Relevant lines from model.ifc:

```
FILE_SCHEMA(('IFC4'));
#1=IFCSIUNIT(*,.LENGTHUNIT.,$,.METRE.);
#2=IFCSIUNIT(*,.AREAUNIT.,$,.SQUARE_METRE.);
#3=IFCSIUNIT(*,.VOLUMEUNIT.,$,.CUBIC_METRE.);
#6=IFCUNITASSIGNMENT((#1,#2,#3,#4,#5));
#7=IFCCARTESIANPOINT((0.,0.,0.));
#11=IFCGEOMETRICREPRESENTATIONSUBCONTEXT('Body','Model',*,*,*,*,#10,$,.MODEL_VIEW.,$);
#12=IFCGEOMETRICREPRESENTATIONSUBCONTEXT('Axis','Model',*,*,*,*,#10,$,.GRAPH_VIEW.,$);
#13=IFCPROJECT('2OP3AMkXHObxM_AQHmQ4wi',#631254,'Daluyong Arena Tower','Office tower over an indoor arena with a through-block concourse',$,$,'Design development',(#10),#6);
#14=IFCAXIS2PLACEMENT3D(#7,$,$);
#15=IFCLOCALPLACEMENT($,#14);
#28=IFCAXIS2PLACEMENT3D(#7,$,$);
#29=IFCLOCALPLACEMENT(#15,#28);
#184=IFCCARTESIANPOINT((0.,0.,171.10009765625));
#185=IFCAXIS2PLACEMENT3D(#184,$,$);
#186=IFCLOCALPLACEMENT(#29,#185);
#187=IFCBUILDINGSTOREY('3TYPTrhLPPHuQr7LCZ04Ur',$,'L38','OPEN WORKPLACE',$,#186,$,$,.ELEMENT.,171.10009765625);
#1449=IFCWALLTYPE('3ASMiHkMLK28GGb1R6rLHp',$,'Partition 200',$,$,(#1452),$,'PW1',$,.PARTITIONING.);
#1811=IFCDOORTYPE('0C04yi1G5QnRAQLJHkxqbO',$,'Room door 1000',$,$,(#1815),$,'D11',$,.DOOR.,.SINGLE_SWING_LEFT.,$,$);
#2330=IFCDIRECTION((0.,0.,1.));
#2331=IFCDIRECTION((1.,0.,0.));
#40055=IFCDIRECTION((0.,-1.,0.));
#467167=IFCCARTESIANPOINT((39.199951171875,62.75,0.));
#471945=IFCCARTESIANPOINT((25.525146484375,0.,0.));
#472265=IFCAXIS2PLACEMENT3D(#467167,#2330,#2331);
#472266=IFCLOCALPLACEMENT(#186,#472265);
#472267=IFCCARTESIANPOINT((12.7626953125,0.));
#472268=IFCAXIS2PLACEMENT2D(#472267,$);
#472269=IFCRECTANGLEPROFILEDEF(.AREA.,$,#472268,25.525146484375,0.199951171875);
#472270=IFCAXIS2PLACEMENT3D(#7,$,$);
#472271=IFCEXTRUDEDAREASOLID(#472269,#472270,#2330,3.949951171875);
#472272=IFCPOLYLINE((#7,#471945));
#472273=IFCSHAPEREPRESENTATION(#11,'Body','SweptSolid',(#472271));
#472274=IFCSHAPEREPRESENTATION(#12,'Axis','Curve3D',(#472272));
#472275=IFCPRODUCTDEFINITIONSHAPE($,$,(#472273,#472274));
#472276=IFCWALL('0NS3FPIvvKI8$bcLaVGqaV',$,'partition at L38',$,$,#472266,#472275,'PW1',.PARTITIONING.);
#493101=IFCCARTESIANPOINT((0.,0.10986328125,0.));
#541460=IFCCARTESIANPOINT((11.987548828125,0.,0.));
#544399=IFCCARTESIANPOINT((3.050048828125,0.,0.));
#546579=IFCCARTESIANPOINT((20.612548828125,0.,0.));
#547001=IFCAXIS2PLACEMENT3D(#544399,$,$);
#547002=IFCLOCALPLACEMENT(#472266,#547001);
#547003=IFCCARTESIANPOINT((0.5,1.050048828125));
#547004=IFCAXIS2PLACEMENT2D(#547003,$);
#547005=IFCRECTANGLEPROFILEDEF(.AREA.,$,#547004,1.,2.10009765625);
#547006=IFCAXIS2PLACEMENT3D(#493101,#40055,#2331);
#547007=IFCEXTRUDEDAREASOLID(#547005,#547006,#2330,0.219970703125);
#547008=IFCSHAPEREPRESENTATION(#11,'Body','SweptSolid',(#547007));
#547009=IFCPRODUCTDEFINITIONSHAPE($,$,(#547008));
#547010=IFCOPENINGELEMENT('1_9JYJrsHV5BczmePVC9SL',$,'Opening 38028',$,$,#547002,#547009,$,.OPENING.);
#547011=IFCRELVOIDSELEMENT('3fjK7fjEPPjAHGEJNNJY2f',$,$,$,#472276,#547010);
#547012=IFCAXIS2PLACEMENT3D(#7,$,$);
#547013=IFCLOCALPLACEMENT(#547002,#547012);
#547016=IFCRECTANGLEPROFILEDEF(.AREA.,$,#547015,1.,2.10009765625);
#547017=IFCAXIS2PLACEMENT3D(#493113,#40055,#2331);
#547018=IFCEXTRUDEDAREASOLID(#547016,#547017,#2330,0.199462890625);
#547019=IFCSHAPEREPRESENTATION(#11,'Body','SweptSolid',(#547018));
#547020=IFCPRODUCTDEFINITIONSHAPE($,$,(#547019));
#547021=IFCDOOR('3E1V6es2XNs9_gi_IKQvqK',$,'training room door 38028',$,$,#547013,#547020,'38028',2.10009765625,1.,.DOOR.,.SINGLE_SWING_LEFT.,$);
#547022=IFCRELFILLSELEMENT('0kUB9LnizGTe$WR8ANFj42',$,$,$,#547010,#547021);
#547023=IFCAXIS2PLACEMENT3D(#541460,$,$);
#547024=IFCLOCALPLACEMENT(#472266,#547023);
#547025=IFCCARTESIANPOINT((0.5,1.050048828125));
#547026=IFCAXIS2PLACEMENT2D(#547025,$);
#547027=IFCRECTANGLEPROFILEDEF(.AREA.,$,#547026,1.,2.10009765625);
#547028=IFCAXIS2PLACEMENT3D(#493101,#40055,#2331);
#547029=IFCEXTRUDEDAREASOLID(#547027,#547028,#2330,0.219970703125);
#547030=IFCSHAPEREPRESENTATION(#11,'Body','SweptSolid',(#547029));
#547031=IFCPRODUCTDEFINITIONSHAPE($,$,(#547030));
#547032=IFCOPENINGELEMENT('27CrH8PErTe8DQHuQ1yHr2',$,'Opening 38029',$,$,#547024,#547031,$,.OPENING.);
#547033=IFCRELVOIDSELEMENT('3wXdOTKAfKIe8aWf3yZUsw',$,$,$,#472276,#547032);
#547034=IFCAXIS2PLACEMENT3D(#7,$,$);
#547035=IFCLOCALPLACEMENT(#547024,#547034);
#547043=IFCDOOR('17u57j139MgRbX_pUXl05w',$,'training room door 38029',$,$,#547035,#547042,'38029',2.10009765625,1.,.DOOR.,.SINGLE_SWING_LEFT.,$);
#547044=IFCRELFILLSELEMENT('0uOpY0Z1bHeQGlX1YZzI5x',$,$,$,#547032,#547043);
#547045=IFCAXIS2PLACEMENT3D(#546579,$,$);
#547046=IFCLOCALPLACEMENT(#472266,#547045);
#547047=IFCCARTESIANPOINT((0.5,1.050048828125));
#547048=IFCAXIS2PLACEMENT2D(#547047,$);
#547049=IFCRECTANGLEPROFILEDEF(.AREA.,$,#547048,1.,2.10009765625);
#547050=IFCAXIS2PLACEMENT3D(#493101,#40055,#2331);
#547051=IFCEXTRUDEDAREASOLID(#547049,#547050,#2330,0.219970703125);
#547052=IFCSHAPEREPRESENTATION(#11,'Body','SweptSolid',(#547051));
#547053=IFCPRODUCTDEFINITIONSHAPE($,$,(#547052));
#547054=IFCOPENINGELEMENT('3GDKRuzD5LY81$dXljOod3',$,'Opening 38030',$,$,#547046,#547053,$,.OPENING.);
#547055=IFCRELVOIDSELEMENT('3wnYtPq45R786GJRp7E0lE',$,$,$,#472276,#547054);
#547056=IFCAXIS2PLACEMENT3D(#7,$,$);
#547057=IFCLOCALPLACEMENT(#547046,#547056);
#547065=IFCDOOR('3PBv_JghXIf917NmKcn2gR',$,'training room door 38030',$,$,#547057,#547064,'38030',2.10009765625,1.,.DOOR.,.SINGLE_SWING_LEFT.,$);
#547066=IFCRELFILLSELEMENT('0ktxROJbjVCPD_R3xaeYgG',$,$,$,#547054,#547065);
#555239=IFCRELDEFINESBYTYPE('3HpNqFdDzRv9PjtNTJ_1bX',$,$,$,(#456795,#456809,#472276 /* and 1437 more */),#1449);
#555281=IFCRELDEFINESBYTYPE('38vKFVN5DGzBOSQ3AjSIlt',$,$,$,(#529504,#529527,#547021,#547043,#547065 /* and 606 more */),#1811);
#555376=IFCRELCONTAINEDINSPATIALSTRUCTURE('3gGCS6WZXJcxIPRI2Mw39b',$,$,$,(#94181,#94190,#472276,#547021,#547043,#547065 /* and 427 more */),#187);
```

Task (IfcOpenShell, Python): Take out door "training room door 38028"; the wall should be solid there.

```python
import ifcopenshell
import ifcopenshell.api.feature
import ifcopenshell.api.root
import ifcopenshell.geom
import ifcopenshell.util.shape

model = ifcopenshell.open("model.ifc")
settings = ifcopenshell.geom.settings()


def volume(element):
    """Net volume in cubic metres, openings subtracted."""
    shape = ifcopenshell.geom.create_shape(settings, element)
    return ifcopenshell.util.shape.get_volume(shape.geometry)


door = model.by_guid("3E1V6es2XNs9_gi_IKQvqK")
opening = door.FillsVoids[0].RelatingOpeningElement
wall = opening.VoidsElements[0].RelatingBuildingElement
before = volume(wall)

ifcopenshell.api.root.remove_product(model, product=door)
ifcopenshell.api.feature.remove_feature(model, feature=opening)

after = volume(wall)

print(f"wall volume {before:.3f} -> {after:.3f} m3")

model.write("model_updated.ifc")
```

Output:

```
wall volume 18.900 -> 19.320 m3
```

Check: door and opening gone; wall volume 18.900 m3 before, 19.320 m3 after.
